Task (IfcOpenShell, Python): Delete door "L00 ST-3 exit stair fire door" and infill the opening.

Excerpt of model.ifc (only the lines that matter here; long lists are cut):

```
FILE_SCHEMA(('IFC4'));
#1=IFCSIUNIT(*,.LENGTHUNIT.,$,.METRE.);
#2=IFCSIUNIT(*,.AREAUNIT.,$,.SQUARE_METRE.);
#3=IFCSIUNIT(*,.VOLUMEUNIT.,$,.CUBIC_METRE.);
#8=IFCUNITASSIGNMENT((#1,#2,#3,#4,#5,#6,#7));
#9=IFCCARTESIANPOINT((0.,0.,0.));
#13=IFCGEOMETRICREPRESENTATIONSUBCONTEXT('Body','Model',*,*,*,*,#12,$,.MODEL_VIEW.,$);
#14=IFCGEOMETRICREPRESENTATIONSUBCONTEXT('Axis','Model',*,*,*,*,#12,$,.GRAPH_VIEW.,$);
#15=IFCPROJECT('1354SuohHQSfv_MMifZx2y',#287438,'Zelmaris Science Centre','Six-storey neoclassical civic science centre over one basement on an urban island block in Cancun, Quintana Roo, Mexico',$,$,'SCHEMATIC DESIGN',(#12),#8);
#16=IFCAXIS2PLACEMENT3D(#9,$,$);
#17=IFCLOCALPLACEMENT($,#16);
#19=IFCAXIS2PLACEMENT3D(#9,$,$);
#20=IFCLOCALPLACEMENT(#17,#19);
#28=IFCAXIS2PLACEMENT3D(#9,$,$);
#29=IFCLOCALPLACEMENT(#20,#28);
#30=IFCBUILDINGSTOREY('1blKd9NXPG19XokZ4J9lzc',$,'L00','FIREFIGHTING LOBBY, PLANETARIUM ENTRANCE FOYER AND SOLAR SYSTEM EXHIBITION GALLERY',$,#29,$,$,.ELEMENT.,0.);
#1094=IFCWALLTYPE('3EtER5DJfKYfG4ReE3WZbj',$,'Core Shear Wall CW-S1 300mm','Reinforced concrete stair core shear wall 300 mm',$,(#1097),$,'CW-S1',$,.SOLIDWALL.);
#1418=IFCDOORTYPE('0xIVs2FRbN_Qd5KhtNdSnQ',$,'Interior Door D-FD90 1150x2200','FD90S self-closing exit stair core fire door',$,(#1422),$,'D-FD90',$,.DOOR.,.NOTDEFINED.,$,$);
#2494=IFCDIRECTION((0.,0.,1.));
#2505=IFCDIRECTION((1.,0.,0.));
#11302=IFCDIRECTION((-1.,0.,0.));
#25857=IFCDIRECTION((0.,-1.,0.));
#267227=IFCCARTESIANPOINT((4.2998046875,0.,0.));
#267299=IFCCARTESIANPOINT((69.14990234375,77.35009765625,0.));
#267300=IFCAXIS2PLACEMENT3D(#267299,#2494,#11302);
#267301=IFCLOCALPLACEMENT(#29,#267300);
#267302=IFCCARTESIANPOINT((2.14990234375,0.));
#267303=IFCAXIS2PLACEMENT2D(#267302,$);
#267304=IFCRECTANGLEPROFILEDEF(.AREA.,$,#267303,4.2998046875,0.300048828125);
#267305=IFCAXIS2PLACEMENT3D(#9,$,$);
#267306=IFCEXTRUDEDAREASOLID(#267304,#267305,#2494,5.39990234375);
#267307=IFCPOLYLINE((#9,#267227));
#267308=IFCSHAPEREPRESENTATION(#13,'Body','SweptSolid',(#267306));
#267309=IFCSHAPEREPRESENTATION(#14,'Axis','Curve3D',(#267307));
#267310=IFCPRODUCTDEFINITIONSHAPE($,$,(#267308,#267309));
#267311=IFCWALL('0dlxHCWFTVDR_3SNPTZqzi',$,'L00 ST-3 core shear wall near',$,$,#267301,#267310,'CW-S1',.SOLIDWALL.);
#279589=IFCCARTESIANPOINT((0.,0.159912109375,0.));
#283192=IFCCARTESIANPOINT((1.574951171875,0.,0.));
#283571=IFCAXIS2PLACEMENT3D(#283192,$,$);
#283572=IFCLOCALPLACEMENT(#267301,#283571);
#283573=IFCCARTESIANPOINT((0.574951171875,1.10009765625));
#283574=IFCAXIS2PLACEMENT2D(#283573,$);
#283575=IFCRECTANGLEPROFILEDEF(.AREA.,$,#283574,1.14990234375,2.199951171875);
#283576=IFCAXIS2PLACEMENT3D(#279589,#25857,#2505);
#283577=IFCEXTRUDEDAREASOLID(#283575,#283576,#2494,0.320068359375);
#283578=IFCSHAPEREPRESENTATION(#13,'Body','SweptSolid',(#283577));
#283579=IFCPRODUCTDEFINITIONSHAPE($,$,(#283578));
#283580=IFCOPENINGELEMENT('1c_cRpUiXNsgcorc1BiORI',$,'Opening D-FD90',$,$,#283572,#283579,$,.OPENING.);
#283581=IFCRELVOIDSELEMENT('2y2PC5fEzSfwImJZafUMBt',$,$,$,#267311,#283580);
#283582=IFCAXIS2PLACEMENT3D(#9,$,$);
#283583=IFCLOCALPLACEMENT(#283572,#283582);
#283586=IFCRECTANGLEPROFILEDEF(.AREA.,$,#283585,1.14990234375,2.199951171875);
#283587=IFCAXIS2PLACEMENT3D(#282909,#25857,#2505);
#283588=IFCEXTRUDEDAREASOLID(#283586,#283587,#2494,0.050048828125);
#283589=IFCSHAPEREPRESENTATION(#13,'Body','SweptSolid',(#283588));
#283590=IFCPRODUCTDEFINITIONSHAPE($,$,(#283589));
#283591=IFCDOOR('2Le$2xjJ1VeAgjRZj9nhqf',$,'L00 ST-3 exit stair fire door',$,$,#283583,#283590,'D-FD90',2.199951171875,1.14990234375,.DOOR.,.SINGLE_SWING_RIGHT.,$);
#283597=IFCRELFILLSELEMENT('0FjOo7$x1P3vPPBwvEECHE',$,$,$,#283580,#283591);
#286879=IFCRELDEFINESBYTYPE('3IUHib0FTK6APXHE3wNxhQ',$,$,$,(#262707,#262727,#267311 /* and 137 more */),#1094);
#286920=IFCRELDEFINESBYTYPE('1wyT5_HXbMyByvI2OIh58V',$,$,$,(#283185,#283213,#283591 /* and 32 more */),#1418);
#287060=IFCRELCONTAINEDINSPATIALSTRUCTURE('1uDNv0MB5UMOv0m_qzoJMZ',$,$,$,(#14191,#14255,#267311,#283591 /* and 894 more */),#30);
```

```python
import ifcopenshell
import ifcopenshell.api.feature
import ifcopenshell.api.root
import ifcopenshell.geom
import ifcopenshell.util.shape

model = ifcopenshell.open("model.ifc")
settings = ifcopenshell.geom.settings()


def volume(element):
    """Net volume in cubic metres, openings subtracted."""
    shape = ifcopenshell.geom.create_shape(settings, element)
    return ifcopenshell.util.shape.get_volume(shape.geometry)


door = model.by_guid("2Le$2xjJ1VeAgjRZj9nhqf")
opening = door.FillsVoids[0].RelatingOpeningElement
wall = opening.VoidsElements[0].RelatingBuildingElement
before = volume(wall)

ifcopenshell.api.root.remove_product(model, product=door)
ifcopenshell.api.feature.remove_feature(model, feature=opening)

after = volume(wall)

print(f"wall volume {before:.3f} -> {after:.3f} m3")

model.write("model_edited.ifc")
```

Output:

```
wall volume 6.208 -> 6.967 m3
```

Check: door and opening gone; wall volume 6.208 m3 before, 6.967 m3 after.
